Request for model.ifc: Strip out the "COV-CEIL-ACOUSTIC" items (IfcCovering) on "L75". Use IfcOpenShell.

First a look at what the model holds.

```python
import ifcopenshell
import ifcopenshell.util.element

model = ifcopenshell.open("model.ifc")
print(model.schema)
storey = next(s for s in model.by_type("IfcBuildingStorey") if s.Name == "L75")
coverings = [e for e in ifcopenshell.util.element.get_decomposition(storey) if e.is_a("IfcCovering")]
seen = {}
for e in coverings:
    element_type = ifcopenshell.util.element.get_type(e)
    name = element_type.Name if element_type not in (None, e) else None
    seen[name] = seen.get(name, 0) + 1
for name, count in sorted(seen.items(), key=str):
    print(count, "x", name)
```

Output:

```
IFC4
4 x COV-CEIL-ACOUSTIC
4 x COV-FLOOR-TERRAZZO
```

```python
import ifcopenshell
import ifcopenshell.api.root
import ifcopenshell.util.element

model = ifcopenshell.open("model.ifc")

storey = next(s for s in model.by_type("IfcBuildingStorey") if s.Name == "L75")
coverings = [e for e in ifcopenshell.util.element.get_decomposition(storey) if e.is_a("IfcCovering")]
targets = [e for e in coverings if (t := ifcopenshell.util.element.get_type(e)) not in (None, e) and t.Name == "COV-CEIL-ACOUSTIC"]

for e in targets:
    ifcopenshell.api.root.remove_product(model, product=e)
print(len(targets), "removed")

model.write("model-out.ifc")
```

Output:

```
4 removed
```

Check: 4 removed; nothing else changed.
